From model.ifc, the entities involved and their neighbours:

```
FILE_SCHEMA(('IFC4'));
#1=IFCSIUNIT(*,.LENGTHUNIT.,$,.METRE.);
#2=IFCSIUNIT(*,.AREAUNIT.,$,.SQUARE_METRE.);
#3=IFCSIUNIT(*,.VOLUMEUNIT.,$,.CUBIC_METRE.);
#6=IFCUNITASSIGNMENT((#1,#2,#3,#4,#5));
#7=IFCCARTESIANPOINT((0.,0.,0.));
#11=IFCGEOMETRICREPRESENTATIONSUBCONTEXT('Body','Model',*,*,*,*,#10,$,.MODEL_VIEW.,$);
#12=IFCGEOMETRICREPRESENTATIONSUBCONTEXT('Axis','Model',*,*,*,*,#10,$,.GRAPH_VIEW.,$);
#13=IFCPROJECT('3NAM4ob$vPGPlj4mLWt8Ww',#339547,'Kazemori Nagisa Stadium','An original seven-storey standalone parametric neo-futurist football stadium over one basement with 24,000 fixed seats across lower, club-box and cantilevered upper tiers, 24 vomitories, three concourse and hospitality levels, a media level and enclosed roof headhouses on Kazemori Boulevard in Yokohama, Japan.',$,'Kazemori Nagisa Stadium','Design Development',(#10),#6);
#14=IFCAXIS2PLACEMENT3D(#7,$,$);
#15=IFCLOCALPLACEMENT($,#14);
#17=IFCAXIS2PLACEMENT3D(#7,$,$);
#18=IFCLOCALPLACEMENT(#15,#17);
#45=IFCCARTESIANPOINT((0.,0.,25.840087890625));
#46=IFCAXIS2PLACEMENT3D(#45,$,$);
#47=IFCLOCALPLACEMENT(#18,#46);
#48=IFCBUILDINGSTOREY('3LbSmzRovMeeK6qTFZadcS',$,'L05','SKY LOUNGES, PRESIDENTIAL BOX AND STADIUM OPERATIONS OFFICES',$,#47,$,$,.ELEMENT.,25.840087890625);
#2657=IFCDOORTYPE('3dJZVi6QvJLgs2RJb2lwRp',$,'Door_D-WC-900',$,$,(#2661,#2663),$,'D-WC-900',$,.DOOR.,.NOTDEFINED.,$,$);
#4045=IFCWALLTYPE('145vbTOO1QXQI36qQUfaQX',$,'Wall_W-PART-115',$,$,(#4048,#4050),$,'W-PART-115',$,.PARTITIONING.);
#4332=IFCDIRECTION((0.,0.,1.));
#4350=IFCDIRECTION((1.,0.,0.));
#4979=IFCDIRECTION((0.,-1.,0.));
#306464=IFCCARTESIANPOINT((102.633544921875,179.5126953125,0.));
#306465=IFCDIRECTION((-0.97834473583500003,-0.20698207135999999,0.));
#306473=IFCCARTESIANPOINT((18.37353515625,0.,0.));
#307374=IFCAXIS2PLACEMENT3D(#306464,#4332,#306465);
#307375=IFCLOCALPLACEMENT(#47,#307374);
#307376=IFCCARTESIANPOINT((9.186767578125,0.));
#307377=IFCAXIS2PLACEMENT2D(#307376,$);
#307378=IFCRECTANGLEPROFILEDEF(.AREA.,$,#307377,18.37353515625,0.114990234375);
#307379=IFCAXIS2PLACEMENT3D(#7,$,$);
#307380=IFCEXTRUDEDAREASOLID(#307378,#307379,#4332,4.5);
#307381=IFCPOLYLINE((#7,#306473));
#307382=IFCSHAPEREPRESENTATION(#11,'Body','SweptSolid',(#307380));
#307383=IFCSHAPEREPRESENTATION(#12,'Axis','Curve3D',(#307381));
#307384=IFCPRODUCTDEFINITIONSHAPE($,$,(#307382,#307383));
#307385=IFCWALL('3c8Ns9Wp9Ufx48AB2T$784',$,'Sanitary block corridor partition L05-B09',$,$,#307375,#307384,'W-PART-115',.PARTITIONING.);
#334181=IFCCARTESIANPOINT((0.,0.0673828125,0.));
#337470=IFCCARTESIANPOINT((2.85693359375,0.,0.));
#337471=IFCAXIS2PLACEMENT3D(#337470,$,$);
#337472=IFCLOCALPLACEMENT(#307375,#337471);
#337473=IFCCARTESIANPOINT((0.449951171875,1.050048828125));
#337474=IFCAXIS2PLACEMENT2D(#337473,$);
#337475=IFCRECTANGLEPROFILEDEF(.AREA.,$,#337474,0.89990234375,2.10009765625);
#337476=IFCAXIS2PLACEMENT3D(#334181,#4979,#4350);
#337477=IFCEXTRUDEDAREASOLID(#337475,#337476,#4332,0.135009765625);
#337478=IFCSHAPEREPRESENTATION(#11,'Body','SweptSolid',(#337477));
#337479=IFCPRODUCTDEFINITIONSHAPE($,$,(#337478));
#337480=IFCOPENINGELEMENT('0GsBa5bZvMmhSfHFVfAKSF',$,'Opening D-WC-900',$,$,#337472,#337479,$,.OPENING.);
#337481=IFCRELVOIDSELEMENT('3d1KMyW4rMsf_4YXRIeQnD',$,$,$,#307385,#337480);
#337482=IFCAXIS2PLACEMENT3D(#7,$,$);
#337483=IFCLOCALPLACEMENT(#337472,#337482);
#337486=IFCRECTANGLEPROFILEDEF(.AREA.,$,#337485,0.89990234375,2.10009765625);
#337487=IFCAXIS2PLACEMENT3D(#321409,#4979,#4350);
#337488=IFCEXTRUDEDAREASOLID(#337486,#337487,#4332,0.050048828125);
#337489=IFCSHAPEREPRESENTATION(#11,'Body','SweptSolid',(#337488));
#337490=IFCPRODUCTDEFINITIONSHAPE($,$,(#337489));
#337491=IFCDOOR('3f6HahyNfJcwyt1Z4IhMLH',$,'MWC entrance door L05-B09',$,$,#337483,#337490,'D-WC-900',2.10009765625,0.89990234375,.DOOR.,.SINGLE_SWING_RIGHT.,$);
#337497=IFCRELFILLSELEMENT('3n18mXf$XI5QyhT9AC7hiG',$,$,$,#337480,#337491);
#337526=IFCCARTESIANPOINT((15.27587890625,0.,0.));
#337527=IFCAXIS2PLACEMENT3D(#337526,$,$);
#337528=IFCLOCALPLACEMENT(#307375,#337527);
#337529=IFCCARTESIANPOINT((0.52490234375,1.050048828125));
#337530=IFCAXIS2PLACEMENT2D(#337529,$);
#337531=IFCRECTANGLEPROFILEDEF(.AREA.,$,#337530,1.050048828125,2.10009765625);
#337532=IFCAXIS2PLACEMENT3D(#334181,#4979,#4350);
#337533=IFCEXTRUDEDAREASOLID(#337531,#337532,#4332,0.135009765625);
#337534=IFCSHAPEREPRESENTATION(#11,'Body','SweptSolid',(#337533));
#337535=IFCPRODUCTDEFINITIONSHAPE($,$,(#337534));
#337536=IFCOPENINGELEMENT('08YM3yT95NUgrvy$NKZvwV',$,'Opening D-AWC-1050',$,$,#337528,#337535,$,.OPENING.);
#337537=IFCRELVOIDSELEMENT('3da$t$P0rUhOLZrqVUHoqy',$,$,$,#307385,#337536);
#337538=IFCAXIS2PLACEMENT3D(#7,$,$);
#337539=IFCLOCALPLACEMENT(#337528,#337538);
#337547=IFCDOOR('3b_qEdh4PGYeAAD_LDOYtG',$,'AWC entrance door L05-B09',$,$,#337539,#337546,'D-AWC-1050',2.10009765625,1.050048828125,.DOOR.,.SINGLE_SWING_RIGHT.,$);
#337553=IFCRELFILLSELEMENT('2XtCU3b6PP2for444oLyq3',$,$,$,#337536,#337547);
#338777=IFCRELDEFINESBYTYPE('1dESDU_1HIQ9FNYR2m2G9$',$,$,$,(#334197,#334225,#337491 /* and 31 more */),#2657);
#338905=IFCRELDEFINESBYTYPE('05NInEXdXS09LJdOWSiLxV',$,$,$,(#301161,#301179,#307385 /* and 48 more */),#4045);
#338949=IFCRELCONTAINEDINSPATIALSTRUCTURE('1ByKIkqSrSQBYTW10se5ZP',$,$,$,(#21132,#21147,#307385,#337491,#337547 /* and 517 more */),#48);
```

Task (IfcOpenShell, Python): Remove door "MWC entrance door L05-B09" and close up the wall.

```python
import ifcopenshell
import ifcopenshell.api.feature
import ifcopenshell.api.root
import ifcopenshell.geom
import ifcopenshell.util.shape

model = ifcopenshell.open("model.ifc")
settings = ifcopenshell.geom.settings()


def volume(element):
    """Net volume in cubic metres, openings subtracted."""
    shape = ifcopenshell.geom.create_shape(settings, element)
    return ifcopenshell.util.shape.get_volume(shape.geometry)


door = model.by_guid("3f6HahyNfJcwyt1Z4IhMLH")
opening = door.FillsVoids[0].RelatingOpeningElement
wall = opening.VoidsElements[0].RelatingBuildingElement
before = volume(wall)

ifcopenshell.api.root.remove_product(model, product=door)
ifcopenshell.api.feature.remove_feature(model, feature=opening)

after = volume(wall)

print(f"wall volume {before:.3f} -> {after:.3f} m3")

model.write("model_edited.ifc")
```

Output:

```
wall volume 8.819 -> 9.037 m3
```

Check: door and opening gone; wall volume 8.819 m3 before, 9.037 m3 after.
